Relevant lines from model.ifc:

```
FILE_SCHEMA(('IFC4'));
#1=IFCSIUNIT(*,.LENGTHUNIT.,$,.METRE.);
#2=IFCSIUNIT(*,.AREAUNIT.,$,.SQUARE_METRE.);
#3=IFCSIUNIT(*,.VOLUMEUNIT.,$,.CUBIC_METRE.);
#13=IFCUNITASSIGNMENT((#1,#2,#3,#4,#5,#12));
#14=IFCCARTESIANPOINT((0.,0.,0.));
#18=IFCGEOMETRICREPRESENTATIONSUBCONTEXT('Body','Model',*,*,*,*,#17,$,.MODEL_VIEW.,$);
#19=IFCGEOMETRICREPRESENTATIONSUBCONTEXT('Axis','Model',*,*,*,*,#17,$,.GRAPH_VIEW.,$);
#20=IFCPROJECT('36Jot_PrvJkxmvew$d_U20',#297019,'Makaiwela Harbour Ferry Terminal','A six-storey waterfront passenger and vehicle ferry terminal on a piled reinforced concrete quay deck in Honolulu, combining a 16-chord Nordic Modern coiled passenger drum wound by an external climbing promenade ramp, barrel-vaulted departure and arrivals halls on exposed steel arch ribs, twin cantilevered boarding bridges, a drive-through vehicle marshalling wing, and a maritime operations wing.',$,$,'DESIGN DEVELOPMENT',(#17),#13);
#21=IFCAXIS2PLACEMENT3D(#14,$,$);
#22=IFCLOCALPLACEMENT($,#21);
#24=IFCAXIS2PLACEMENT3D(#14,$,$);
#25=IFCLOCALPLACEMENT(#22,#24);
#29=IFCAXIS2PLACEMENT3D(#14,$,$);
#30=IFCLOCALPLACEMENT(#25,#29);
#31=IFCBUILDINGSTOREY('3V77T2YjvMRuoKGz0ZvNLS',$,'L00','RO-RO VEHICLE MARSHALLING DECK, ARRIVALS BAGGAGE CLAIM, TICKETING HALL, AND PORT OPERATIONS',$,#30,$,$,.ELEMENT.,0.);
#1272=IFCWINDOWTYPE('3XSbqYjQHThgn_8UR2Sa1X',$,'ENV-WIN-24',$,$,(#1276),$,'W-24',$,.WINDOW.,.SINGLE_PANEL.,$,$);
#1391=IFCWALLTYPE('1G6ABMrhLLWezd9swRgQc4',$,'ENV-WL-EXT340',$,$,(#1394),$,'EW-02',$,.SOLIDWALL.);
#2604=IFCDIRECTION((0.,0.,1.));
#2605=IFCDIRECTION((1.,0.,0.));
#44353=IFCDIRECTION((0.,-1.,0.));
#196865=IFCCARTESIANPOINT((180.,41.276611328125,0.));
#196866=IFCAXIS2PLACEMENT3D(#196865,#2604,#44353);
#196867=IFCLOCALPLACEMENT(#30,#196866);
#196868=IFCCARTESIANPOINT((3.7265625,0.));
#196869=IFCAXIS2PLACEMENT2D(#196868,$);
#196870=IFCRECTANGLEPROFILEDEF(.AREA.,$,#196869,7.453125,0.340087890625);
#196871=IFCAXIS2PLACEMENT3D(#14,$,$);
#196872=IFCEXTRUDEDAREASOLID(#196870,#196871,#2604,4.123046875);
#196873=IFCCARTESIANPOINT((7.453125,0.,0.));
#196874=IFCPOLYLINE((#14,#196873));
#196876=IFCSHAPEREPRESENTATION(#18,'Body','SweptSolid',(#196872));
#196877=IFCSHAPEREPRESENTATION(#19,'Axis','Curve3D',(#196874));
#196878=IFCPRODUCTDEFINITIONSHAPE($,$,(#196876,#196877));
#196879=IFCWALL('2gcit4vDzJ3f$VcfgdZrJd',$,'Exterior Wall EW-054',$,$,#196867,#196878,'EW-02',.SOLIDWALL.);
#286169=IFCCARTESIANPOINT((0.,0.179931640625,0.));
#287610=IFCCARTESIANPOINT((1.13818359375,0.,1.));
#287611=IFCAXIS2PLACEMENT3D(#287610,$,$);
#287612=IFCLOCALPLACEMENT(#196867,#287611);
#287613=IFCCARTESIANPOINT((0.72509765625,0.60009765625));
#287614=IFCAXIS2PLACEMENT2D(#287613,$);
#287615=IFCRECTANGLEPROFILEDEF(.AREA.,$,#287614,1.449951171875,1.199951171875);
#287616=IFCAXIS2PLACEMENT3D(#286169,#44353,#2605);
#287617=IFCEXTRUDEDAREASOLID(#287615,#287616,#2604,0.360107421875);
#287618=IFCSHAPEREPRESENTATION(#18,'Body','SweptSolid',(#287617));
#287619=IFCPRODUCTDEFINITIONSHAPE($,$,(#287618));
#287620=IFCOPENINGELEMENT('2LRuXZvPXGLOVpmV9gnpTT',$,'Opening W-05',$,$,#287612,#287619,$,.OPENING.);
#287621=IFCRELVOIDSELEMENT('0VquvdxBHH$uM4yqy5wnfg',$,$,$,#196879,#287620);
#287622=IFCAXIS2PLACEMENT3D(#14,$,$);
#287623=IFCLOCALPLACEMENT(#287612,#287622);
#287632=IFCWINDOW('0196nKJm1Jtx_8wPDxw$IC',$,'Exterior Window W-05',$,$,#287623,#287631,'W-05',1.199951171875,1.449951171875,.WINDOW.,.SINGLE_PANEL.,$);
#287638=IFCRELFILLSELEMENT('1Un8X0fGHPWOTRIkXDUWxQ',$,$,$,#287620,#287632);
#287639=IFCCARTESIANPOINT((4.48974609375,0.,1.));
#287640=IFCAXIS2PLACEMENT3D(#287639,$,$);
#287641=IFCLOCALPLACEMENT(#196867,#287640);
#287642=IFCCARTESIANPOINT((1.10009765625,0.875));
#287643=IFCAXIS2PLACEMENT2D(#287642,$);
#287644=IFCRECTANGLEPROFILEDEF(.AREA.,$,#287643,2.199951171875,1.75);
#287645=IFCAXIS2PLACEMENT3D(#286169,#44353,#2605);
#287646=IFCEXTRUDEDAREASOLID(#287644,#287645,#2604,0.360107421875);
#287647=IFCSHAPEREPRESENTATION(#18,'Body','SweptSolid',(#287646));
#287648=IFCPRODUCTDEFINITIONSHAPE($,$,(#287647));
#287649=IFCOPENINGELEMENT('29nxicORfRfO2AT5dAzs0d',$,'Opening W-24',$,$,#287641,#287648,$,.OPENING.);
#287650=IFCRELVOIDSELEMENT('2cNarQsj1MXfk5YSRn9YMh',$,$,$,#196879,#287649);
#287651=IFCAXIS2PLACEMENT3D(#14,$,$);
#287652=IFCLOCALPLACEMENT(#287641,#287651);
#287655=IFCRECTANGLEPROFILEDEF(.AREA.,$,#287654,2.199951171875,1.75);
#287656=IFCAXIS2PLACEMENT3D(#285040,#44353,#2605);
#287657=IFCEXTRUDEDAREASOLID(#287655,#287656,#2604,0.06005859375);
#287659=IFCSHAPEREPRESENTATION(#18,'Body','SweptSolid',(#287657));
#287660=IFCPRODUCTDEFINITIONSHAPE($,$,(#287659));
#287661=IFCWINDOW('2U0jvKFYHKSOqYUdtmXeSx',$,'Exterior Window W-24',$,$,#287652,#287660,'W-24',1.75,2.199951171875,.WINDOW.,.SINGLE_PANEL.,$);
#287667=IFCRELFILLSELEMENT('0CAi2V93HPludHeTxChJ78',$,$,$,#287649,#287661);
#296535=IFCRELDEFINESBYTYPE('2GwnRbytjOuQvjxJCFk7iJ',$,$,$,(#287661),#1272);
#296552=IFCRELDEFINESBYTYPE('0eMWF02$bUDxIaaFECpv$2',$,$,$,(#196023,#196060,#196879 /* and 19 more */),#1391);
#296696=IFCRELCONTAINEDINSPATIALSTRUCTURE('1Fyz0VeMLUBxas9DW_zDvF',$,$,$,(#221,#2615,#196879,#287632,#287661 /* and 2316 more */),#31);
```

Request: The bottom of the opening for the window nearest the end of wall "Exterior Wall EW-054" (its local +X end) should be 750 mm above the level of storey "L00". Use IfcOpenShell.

```python
import numpy as np
import ifcopenshell
import ifcopenshell.api.geometry
import ifcopenshell.geom
import ifcopenshell.util.element
import ifcopenshell.util.placement
import ifcopenshell.util.shape
import ifcopenshell.util.unit

model = ifcopenshell.open("model.ifc")
unit_scale = ifcopenshell.util.unit.calculate_unit_scale(model)

window = model.by_id(287661)
opening = window.FillsVoids[0].RelatingOpeningElement
storey = ifcopenshell.util.element.get_container(window, ifc_class="IfcBuildingStorey")
level = ifcopenshell.util.placement.get_local_placement(storey.ObjectPlacement)[2, 3]

# The opening's origin need not be at the sill, so measure its lowest point.
shape = ifcopenshell.geom.create_shape(ifcopenshell.geom.settings(), opening)
bottom = ifcopenshell.util.shape.get_shape_bottom_elevation(shape, shape.geometry) / unit_scale
dz = level + 0.75 - bottom

shift = np.array([0.0, 0.0, dz])
# The window is placed relative to its opening, so it follows when the opening moves.
matrix = ifcopenshell.util.placement.get_local_placement(opening.ObjectPlacement)
matrix[:3, 3] += shift
ifcopenshell.api.geometry.edit_object_placement(
    model, product=opening, matrix=matrix, is_si=False, should_transform_children=True
)

print(f"moved by {dz * unit_scale:+.3f} m")

model.write("model-out.ifc")
```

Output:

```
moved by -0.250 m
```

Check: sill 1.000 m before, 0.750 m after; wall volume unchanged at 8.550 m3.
